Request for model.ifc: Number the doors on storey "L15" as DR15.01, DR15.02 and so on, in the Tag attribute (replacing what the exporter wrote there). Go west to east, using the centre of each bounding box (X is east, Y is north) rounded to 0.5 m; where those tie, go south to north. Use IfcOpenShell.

First a look at what the model holds.

```python
import ifcopenshell
import ifcopenshell.util.element
import ifcopenshell.util.placement

model = ifcopenshell.open("model.ifc")
print(model.schema)
storey = next(s for s in model.by_type("IfcBuildingStorey") if s.Name == "L15")
doors = [e for e in ifcopenshell.util.element.get_decomposition(storey) if e.is_a("IfcDoor")]
for e in sorted(doors, key=lambda e: e.id()):
    origin = ifcopenshell.util.placement.get_local_placement(e.ObjectPlacement)[:3, 3]
    print(e.id(), e.Tag, e.Name, origin.round(2) + 0.0, sep=" | ")
```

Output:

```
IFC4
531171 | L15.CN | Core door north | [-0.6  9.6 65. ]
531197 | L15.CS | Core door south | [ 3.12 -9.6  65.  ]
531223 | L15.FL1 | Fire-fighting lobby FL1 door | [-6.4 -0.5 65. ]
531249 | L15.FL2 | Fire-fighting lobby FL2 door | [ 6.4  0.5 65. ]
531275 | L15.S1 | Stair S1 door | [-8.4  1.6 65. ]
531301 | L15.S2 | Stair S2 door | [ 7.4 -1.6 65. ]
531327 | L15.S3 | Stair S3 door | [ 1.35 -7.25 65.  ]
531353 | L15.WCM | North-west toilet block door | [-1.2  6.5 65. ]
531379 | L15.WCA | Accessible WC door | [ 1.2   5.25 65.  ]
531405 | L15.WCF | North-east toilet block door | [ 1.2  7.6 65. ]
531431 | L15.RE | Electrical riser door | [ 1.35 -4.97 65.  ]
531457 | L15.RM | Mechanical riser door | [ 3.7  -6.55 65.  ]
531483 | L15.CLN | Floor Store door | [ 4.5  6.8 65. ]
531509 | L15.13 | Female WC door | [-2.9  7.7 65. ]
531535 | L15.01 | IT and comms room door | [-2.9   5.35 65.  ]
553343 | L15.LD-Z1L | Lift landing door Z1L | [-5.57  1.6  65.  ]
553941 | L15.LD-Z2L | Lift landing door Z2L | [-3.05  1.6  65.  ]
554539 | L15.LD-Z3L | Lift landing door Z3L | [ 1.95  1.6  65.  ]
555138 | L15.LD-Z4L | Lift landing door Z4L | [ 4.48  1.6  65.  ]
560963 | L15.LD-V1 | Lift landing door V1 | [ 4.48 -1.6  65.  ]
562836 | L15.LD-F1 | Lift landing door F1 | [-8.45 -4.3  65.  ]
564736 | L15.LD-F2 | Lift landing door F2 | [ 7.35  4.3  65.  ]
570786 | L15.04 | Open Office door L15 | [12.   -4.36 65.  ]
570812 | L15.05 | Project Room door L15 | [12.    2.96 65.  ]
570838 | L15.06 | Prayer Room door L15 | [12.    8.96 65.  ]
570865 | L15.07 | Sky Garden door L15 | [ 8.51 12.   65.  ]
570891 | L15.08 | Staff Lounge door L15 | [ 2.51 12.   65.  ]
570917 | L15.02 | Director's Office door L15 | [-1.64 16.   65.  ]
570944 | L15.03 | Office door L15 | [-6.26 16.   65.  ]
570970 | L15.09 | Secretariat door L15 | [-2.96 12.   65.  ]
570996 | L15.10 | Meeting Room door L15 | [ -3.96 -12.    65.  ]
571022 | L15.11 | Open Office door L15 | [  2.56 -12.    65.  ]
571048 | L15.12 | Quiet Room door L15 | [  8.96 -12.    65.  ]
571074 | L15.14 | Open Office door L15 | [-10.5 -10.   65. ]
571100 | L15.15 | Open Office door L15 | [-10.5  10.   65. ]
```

```python
import ifcopenshell
import ifcopenshell.geom
import ifcopenshell.util.element
import ifcopenshell.util.shape

model = ifcopenshell.open("model.ifc")
settings = ifcopenshell.geom.settings()
settings.set("use-world-coords", True)


def centre(element):
    shape = ifcopenshell.geom.create_shape(settings, element)
    return ifcopenshell.util.shape.get_bbox_centroid(shape.geometry)


storey = next(s for s in model.by_type("IfcBuildingStorey") if s.Name == "L15")
doors = [e for e in ifcopenshell.util.element.get_decomposition(storey) if e.is_a("IfcDoor")]

# Insertion points can sit at a corner or the storey origin, so sort by the geometry (in metres).
centres = {e: centre(e) for e in doors}
doors.sort(key=lambda e: (round(centres[e][0] / 0.5), centres[e][1]))

for i, e in enumerate(doors, start=1):
    number = f"DR15.{i:02d}"
    e.Tag = number
    print(e.id(), number)

model.write("model_v2.ifc")
```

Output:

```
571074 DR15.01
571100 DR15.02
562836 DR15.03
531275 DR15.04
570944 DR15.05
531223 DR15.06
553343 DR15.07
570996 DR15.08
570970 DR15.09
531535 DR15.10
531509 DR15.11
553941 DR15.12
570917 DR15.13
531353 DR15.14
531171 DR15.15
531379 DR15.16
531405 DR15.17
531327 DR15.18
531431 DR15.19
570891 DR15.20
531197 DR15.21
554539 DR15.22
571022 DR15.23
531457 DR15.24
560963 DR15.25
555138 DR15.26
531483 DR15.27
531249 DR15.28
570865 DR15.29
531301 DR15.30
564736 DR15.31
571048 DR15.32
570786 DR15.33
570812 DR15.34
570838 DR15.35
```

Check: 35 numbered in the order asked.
